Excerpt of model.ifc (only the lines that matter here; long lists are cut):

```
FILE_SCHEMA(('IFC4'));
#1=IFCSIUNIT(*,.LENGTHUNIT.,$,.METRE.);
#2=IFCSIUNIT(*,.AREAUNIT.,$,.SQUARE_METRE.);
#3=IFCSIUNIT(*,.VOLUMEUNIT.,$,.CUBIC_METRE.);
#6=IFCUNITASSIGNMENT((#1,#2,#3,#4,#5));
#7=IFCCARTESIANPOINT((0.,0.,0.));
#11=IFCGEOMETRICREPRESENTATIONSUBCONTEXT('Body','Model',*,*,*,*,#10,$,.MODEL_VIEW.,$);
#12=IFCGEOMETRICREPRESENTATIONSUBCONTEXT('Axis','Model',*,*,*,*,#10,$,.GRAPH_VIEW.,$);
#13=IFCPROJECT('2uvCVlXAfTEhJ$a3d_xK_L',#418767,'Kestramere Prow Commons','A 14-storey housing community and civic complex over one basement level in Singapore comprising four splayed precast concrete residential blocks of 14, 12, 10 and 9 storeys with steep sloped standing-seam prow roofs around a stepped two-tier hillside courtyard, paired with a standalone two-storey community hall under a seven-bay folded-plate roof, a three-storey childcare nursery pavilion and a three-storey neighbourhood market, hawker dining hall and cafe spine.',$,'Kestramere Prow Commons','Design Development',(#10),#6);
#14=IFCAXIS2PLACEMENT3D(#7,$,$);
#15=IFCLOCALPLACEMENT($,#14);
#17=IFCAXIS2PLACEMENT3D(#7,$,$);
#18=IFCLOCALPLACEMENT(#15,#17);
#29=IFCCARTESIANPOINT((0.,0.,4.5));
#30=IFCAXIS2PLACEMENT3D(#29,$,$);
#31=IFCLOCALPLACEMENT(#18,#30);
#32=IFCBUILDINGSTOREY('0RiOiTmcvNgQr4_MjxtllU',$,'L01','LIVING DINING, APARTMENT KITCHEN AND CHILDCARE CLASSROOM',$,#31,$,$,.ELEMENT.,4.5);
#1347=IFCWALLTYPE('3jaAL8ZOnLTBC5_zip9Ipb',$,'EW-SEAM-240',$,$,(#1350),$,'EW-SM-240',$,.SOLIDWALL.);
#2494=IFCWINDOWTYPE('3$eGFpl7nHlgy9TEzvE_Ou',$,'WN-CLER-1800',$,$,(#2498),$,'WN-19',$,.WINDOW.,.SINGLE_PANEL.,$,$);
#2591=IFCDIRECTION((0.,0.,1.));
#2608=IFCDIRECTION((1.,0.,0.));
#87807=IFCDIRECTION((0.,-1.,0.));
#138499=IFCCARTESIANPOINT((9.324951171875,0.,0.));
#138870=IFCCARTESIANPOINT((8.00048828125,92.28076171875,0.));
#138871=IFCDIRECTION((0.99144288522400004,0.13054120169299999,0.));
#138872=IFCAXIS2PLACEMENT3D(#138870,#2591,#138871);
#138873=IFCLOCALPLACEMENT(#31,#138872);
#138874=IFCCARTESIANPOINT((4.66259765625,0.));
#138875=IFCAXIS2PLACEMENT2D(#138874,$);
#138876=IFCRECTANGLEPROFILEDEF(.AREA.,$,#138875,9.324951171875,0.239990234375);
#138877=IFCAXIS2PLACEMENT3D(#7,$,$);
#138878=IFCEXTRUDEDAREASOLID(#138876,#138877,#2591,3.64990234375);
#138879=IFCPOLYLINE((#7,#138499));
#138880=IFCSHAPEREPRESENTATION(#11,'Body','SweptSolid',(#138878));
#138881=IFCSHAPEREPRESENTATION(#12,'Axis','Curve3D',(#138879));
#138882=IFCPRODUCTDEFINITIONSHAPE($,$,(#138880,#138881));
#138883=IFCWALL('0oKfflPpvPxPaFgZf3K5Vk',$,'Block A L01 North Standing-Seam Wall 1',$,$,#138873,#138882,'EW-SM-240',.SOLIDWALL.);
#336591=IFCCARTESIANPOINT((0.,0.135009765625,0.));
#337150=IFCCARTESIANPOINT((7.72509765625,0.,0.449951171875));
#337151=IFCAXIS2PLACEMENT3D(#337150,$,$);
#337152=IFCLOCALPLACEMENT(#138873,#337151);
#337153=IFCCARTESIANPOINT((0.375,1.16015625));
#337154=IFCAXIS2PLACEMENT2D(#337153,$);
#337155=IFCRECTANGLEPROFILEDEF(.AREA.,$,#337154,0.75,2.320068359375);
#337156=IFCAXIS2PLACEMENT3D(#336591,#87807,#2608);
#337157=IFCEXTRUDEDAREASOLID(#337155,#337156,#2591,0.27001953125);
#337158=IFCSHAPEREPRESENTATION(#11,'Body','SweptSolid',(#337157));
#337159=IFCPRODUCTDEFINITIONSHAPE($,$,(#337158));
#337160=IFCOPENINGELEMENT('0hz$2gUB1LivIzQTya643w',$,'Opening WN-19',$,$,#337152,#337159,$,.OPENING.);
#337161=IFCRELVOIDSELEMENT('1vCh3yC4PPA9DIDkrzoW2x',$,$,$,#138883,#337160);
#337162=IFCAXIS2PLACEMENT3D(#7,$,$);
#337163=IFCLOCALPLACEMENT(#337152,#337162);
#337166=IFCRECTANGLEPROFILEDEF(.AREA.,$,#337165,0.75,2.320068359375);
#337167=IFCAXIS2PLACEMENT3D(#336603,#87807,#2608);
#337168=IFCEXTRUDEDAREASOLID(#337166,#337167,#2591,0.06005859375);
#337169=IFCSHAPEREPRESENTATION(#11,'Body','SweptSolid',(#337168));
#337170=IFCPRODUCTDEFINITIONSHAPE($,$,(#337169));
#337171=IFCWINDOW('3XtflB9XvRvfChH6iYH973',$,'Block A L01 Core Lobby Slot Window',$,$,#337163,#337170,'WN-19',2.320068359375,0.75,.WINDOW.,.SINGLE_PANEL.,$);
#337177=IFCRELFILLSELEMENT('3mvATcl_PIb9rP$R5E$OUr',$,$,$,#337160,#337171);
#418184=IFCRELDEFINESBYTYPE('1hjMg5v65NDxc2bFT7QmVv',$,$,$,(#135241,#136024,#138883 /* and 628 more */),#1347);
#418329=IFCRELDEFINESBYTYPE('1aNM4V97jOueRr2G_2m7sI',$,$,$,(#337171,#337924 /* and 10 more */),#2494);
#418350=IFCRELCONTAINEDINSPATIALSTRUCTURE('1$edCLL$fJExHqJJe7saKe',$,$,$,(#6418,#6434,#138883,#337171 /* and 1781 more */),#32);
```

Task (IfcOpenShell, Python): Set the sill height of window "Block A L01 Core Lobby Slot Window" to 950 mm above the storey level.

```python
import numpy as np
import ifcopenshell
import ifcopenshell.api.geometry
import ifcopenshell.geom
import ifcopenshell.util.element
import ifcopenshell.util.placement
import ifcopenshell.util.shape
import ifcopenshell.util.unit

model = ifcopenshell.open("model.ifc")
unit_scale = ifcopenshell.util.unit.calculate_unit_scale(model)

window = model.by_id(337171)
opening = window.FillsVoids[0].RelatingOpeningElement
storey = ifcopenshell.util.element.get_container(window, ifc_class="IfcBuildingStorey")
level = ifcopenshell.util.placement.get_local_placement(storey.ObjectPlacement)[2, 3]

# The opening's origin need not be at the sill, so measure its lowest point.
shape = ifcopenshell.geom.create_shape(ifcopenshell.geom.settings(), opening)
bottom = ifcopenshell.util.shape.get_shape_bottom_elevation(shape, shape.geometry) / unit_scale
dz = level + 0.95 / unit_scale - bottom

shift = np.array([0.0, 0.0, dz])
# The window is placed relative to its opening, so it follows when the opening moves.
matrix = ifcopenshell.util.placement.get_local_placement(opening.ObjectPlacement)
matrix[:3, 3] += shift
ifcopenshell.api.geometry.edit_object_placement(
    model, product=opening, matrix=matrix, is_si=False, should_transform_children=True
)

print(f"moved by {dz * unit_scale:+.3f} m")

model.write("model_rev.ifc")
```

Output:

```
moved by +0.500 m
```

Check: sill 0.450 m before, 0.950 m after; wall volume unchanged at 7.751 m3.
